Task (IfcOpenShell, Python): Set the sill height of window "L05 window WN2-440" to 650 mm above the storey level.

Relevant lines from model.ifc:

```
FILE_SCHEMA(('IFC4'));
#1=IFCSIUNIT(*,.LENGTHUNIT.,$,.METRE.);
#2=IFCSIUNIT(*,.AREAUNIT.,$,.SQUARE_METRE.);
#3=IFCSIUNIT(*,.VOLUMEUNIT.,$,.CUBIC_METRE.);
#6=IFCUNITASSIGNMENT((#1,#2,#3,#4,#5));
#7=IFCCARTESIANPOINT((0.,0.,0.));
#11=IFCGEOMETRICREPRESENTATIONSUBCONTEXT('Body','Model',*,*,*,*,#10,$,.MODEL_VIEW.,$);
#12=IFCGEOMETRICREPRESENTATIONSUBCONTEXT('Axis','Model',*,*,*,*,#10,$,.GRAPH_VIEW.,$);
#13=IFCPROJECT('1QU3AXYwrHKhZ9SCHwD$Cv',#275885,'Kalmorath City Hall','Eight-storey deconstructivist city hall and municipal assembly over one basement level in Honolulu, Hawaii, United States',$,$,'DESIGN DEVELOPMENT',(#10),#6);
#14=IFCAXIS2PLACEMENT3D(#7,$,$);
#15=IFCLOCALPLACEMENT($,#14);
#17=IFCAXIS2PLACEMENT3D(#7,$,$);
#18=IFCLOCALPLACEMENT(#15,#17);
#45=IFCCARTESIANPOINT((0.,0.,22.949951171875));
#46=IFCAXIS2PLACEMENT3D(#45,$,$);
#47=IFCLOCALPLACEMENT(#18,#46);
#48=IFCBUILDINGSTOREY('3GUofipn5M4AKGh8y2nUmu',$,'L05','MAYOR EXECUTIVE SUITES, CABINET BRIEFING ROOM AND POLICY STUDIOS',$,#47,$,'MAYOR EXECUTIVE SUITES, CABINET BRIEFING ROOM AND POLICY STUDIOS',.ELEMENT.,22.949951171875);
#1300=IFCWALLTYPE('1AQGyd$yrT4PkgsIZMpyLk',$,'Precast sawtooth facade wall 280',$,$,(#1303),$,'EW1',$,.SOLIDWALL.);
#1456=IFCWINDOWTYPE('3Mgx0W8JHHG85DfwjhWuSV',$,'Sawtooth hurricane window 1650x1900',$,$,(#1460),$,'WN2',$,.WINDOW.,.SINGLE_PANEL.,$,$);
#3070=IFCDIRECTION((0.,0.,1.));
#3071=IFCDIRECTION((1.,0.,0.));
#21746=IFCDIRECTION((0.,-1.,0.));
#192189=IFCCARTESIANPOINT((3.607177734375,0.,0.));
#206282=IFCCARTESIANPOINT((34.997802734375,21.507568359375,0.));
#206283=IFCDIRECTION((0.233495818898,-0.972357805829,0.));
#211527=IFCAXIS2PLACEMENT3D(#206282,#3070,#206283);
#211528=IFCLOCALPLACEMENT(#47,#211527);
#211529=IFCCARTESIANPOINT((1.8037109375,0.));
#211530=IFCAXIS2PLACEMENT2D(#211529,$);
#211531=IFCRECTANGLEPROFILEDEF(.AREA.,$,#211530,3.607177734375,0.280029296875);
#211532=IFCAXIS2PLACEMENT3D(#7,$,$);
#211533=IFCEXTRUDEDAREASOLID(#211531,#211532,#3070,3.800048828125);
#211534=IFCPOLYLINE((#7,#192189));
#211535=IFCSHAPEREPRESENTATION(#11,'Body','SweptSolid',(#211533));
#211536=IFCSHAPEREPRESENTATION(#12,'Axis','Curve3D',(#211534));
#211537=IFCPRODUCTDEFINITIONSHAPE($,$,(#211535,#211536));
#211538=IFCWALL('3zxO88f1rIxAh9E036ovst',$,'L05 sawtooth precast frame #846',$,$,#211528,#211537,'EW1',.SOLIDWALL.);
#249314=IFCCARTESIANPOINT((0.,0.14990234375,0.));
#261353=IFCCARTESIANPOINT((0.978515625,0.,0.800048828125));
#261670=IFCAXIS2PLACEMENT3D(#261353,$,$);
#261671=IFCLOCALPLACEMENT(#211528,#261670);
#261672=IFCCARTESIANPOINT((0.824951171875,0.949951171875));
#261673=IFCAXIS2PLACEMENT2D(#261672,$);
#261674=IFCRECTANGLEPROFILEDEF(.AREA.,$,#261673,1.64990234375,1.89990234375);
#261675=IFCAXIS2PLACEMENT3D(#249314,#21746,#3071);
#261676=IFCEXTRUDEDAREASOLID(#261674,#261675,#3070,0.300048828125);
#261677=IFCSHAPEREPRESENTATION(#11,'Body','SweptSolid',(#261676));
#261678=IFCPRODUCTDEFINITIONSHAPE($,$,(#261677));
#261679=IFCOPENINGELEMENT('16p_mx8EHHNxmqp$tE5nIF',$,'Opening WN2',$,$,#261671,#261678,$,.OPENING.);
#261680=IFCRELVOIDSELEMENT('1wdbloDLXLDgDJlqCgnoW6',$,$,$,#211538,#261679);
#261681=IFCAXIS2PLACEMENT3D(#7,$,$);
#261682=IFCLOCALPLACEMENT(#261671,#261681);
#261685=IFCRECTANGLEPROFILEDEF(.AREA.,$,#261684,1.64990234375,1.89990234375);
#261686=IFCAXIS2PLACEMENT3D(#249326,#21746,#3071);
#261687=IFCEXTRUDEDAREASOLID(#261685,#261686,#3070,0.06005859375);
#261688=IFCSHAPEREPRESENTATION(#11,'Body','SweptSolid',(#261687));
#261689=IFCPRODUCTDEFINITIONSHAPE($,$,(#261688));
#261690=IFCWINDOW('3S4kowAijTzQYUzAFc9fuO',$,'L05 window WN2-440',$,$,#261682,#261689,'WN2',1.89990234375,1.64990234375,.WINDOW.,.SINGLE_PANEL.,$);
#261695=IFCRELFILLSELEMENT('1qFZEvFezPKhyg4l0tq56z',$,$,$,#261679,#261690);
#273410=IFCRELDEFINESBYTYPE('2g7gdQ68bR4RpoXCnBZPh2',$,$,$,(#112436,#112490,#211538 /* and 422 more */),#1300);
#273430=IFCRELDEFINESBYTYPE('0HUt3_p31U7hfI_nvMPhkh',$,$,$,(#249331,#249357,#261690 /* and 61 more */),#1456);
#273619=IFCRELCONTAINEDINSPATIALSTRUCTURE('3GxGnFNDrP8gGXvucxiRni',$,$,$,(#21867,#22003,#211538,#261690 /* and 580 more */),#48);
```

```python
import numpy as np
import ifcopenshell
import ifcopenshell.api.geometry
import ifcopenshell.geom
import ifcopenshell.util.element
import ifcopenshell.util.placement
import ifcopenshell.util.shape
import ifcopenshell.util.unit

model = ifcopenshell.open("model.ifc")
unit_scale = ifcopenshell.util.unit.calculate_unit_scale(model)

window = model.by_guid("3S4kowAijTzQYUzAFc9fuO")
opening = window.FillsVoids[0].RelatingOpeningElement
storey = ifcopenshell.util.element.get_container(window, ifc_class="IfcBuildingStorey")
level = ifcopenshell.util.placement.get_local_placement(storey.ObjectPlacement)[2, 3]

# The opening's origin need not be at the sill, so measure its lowest point.
shape = ifcopenshell.geom.create_shape(ifcopenshell.geom.settings(), opening)
bottom = ifcopenshell.util.shape.get_shape_bottom_elevation(shape, shape.geometry) / unit_scale
dz = level + 0.65 - bottom

shift = np.array([0.0, 0.0, dz])
# The window is placed relative to its opening, so it follows when the opening moves.
matrix = ifcopenshell.util.placement.get_local_placement(opening.ObjectPlacement)
matrix[:3, 3] += shift
ifcopenshell.api.geometry.edit_object_placement(
    model, product=opening, matrix=matrix, is_si=False, should_transform_children=True
)

print(f"moved by {dz * unit_scale:+.3f} m")

model.write("model_rev.ifc")
```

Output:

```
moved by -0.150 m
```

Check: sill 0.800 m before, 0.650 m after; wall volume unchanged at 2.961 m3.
